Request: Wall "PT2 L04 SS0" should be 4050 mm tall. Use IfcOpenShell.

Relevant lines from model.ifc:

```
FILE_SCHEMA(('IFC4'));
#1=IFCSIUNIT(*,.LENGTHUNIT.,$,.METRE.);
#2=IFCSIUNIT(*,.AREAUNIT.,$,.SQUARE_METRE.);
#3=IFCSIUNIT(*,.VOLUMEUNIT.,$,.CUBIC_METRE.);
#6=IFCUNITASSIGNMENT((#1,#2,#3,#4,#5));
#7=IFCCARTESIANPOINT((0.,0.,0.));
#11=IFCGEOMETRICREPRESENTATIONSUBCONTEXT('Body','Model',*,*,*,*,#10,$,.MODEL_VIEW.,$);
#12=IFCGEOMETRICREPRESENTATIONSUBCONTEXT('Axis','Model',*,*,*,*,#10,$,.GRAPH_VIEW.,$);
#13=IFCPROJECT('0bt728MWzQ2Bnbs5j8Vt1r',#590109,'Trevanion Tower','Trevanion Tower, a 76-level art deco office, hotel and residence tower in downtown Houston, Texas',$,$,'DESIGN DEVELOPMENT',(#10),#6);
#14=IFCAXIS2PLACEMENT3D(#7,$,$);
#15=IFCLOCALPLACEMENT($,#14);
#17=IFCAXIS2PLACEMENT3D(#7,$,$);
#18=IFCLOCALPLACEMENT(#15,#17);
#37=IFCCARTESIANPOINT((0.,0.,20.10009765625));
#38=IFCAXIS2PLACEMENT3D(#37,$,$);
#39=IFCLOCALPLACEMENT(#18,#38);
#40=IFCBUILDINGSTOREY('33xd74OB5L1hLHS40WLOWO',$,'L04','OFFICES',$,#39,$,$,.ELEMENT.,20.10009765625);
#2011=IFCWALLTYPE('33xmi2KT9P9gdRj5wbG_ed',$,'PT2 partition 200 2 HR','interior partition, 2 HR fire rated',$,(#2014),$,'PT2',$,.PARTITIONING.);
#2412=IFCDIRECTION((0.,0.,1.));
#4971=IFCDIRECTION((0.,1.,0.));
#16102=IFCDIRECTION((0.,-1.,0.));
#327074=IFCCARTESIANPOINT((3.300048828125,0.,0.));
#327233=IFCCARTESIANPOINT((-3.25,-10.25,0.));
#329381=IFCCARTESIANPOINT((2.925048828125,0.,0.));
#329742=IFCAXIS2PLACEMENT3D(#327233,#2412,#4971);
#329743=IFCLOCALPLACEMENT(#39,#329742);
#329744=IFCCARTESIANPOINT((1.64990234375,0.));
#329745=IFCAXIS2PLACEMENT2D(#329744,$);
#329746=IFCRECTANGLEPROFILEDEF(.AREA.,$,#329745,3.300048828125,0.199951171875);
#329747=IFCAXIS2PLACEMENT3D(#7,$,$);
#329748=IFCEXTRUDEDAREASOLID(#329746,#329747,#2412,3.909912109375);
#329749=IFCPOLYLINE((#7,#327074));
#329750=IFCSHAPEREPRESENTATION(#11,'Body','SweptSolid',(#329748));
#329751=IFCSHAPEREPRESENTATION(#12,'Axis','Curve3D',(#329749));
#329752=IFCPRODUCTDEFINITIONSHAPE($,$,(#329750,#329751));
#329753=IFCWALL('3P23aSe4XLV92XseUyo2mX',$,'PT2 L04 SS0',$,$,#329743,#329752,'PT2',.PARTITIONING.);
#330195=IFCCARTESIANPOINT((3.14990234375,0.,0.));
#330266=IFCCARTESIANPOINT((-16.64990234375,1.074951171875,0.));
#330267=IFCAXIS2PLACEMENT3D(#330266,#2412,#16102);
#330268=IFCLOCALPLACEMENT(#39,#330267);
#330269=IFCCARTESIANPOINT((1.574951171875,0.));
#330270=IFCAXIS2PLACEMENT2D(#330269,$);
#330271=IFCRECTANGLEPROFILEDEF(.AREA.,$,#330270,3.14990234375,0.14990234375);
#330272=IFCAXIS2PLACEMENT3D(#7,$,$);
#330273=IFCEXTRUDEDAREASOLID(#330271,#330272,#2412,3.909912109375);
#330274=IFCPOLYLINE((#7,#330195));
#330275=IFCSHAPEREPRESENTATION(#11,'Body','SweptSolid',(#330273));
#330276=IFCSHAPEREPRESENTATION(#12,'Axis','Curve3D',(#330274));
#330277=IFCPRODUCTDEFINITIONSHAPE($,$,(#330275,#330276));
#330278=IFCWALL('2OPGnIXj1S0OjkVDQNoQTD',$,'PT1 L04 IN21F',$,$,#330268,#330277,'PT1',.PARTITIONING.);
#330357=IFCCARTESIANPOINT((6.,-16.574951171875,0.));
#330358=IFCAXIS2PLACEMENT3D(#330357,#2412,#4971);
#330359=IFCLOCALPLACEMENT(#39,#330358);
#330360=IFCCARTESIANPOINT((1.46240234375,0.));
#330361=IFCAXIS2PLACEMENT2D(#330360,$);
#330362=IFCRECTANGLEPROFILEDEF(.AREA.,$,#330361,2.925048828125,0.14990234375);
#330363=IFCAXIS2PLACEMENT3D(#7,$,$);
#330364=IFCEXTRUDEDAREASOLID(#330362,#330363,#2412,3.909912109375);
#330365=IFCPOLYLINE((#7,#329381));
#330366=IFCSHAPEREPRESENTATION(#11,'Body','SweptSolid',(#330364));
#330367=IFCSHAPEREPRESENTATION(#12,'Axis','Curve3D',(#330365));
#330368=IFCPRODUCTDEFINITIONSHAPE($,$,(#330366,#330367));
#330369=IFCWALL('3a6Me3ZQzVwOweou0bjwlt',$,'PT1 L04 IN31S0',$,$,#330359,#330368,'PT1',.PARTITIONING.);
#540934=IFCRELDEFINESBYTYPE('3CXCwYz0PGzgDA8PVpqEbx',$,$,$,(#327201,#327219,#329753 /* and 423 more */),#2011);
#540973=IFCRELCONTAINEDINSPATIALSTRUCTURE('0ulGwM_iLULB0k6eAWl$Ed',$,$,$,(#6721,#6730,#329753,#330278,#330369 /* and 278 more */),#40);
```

```python
import ifcopenshell
import ifcopenshell.geom
import ifcopenshell.util.representation
import ifcopenshell.util.shape

model = ifcopenshell.open("model.ifc")
settings = ifcopenshell.geom.settings()


def volume(element):
    """Net volume in cubic metres, openings subtracted."""
    shape = ifcopenshell.geom.create_shape(settings, element)
    return ifcopenshell.util.shape.get_volume(shape.geometry)


wall = model.by_guid("3P23aSe4XLV92XseUyo2mX")
before = volume(wall)

body = ifcopenshell.util.representation.get_representation(wall, "Model", "Body")
solid = body.Items[0]
old_height = solid.Depth
solid.Depth = 4.05
after = volume(wall)

print(f"height {old_height:g} -> {solid.Depth:g}, volume {before:.3f} -> {after:.3f} m3")

model.write("model_rev.ifc")
```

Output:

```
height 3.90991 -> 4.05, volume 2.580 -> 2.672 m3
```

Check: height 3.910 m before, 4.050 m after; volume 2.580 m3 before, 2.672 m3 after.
